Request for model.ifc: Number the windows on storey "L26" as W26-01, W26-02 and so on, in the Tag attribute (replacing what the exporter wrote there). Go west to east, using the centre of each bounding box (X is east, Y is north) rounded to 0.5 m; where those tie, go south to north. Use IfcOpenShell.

First a look at what the model holds.

```python
import ifcopenshell
import ifcopenshell.util.element
import ifcopenshell.util.placement

model = ifcopenshell.open("model.ifc")
print(model.schema)
storey = next(s for s in model.by_type("IfcBuildingStorey") if s.Name == "L26")
windows = [e for e in ifcopenshell.util.element.get_decomposition(storey) if e.is_a("IfcWindow")]
for e in sorted(windows, key=lambda e: e.id()):
    origin = ifcopenshell.util.placement.get_local_placement(e.ObjectPlacement)[:3, 3]
    print(e.id(), e.Tag, e.Name, origin.round(2) + 0.0, sep=" | ")
```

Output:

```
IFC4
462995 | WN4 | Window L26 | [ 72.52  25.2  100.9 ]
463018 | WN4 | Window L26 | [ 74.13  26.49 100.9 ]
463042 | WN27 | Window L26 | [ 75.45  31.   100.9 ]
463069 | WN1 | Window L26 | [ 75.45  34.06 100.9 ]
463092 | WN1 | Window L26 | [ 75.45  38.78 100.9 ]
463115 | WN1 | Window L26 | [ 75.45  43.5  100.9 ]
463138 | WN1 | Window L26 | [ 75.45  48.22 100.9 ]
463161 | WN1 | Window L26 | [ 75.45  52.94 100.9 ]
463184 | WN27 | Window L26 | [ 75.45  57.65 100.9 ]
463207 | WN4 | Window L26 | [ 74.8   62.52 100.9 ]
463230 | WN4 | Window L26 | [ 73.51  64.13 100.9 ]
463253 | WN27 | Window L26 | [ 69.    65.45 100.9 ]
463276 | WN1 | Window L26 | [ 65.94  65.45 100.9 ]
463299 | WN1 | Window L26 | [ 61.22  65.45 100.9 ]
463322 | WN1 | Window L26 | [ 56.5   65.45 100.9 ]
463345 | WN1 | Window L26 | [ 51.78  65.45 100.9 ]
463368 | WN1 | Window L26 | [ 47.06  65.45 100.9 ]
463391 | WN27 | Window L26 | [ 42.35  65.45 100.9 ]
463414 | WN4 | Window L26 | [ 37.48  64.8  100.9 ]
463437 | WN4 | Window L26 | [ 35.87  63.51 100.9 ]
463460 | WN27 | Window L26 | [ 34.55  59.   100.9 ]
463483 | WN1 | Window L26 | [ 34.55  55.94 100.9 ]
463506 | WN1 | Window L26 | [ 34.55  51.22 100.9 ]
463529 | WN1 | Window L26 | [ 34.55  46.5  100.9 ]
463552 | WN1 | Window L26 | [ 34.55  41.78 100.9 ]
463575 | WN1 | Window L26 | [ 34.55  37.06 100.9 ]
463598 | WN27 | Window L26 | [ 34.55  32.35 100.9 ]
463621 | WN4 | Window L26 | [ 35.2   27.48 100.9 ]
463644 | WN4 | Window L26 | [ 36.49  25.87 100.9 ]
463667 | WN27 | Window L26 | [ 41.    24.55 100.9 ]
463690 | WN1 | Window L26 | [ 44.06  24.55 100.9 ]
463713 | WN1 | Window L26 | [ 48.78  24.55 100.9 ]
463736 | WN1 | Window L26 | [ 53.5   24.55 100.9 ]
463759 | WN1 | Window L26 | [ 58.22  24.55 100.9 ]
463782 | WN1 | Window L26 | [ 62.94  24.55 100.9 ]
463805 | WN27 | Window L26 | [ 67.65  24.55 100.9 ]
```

```python
import ifcopenshell
import ifcopenshell.geom
import ifcopenshell.util.element
import ifcopenshell.util.shape

model = ifcopenshell.open("model.ifc")
settings = ifcopenshell.geom.settings()
settings.set("use-world-coords", True)


def centre(element):
    shape = ifcopenshell.geom.create_shape(settings, element)
    return ifcopenshell.util.shape.get_bbox_centroid(shape.geometry)


storey = next(s for s in model.by_type("IfcBuildingStorey") if s.Name == "L26")
windows = [e for e in ifcopenshell.util.element.get_decomposition(storey) if e.is_a("IfcWindow")]

# Insertion points can sit at a corner or the storey origin, so sort by the geometry (in metres).
centres = {e: centre(e) for e in windows}
windows.sort(key=lambda e: (round(centres[e][0] / 0.5), centres[e][1]))

for i, e in enumerate(windows, start=1):
    number = f"W26-{i:02d}"
    e.Tag = number
    print(e.id(), number)

model.write("model-out.ifc")
```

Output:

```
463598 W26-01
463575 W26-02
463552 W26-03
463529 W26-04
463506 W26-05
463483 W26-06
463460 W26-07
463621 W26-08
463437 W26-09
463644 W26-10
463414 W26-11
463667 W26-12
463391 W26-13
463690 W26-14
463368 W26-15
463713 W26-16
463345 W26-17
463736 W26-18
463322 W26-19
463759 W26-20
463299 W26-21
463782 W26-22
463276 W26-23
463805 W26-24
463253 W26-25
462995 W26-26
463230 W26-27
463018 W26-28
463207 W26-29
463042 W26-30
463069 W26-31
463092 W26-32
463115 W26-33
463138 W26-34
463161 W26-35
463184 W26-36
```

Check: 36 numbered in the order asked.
